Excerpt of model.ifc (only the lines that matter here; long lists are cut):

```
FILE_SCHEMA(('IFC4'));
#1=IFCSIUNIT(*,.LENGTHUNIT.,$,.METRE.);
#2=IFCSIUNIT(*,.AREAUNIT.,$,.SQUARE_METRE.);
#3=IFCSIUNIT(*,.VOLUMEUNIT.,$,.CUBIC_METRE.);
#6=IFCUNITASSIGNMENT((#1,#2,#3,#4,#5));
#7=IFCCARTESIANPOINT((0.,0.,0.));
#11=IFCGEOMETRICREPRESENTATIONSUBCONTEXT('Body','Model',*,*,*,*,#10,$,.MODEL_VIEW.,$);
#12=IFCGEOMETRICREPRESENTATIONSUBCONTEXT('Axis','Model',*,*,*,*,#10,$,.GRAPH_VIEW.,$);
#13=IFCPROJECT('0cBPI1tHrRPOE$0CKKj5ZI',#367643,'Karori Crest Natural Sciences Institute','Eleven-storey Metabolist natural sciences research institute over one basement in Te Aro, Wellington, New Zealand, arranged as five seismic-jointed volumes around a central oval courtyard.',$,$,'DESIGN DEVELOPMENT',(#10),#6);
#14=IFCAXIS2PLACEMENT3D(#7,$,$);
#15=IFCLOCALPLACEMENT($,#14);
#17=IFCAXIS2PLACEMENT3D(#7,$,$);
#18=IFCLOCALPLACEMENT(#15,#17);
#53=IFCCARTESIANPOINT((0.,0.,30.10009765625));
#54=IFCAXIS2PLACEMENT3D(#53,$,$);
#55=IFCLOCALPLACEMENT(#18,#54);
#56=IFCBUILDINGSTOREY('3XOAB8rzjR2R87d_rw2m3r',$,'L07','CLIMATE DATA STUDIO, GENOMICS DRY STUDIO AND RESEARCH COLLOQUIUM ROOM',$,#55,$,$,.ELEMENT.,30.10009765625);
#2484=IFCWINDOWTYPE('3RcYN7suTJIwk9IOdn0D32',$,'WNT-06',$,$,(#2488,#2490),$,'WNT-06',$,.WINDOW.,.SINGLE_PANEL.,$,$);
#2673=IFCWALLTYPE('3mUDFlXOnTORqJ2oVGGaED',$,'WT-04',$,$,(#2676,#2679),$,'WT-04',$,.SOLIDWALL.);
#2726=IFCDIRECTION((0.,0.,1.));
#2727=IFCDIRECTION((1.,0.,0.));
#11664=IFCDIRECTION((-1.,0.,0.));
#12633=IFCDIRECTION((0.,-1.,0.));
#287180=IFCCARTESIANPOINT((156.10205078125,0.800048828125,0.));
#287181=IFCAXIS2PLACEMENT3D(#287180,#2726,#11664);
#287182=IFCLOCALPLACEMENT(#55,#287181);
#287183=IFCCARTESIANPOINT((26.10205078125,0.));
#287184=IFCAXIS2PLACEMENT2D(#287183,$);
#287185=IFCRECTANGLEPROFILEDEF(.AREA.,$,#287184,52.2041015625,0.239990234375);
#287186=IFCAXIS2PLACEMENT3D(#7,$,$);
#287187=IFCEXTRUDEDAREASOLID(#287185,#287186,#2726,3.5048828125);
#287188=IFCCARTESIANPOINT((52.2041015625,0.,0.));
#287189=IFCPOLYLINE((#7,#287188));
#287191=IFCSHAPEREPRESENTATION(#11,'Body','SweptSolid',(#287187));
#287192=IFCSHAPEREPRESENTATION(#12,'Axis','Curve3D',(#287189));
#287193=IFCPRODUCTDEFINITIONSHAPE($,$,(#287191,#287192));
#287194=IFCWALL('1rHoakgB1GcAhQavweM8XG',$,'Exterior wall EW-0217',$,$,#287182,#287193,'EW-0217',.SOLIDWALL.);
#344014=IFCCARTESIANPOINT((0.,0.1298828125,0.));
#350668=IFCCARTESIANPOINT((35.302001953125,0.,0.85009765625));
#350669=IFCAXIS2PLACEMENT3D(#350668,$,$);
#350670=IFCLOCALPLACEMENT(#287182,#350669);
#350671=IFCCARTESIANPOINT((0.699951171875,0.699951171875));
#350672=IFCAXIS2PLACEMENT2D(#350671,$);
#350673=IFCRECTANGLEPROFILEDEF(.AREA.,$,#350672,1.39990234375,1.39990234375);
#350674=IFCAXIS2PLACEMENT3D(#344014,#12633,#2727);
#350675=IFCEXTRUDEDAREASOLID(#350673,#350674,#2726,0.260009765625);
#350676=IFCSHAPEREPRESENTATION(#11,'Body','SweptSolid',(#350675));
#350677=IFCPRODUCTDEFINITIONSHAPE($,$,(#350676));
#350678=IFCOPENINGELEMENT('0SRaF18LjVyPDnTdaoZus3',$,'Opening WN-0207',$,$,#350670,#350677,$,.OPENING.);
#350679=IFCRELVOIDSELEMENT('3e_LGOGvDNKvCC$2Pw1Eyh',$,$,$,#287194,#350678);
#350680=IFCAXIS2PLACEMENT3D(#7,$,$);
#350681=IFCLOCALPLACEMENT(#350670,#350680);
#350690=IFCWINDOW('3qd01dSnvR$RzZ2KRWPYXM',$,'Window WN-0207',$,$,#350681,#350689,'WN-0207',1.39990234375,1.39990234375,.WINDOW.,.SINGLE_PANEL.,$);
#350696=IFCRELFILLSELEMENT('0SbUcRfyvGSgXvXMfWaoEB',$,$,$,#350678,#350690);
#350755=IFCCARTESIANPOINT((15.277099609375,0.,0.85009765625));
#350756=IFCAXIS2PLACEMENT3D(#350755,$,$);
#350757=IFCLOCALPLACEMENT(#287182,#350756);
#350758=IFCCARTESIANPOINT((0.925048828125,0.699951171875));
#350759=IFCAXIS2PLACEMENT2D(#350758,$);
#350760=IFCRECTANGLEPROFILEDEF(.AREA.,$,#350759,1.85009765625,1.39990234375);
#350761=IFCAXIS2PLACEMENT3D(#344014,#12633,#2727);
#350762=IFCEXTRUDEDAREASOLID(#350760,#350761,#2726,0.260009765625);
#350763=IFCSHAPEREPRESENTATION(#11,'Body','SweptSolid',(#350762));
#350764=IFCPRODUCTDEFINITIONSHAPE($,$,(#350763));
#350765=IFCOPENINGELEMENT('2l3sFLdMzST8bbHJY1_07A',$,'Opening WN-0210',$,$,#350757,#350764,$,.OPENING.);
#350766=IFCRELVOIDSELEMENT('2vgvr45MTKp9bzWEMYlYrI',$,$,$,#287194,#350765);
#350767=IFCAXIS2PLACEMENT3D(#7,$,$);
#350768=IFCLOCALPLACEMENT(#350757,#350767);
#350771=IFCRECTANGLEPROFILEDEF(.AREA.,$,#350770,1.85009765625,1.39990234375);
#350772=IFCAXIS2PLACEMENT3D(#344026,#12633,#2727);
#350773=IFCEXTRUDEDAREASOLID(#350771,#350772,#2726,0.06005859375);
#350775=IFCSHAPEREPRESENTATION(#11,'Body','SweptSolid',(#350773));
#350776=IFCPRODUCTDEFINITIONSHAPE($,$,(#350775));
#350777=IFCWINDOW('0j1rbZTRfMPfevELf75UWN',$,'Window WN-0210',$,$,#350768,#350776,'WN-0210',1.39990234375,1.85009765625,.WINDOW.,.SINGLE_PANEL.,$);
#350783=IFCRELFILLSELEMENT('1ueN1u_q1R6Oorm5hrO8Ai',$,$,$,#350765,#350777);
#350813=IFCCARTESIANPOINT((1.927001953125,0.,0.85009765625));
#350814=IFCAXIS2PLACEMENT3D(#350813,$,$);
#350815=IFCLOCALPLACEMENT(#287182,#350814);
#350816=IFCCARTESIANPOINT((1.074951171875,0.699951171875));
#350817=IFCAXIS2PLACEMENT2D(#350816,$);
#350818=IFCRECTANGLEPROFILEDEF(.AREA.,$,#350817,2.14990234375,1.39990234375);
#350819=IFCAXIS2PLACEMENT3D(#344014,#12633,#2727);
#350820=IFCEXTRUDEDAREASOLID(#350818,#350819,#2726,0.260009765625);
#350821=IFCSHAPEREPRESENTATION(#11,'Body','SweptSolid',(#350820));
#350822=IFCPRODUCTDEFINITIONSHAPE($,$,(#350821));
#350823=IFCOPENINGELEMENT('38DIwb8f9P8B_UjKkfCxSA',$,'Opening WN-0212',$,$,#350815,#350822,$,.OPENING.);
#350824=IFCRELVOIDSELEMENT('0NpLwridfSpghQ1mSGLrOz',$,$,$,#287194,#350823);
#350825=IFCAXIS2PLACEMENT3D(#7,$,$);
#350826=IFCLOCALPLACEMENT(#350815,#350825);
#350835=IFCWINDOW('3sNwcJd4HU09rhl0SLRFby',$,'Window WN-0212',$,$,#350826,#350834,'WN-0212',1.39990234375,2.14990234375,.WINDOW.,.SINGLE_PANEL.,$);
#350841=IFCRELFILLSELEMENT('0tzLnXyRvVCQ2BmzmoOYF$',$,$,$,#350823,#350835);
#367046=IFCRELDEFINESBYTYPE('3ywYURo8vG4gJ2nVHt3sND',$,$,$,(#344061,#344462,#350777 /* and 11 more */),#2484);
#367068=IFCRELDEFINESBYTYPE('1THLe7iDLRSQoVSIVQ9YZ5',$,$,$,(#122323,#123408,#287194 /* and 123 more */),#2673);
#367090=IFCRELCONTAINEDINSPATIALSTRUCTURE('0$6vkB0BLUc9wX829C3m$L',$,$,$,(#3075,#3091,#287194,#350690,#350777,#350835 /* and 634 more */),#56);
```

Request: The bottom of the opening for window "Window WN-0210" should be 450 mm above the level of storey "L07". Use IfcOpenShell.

```python
import numpy as np
import ifcopenshell
import ifcopenshell.api.geometry
import ifcopenshell.geom
import ifcopenshell.util.element
import ifcopenshell.util.placement
import ifcopenshell.util.shape
import ifcopenshell.util.unit

model = ifcopenshell.open("model.ifc")
unit_scale = ifcopenshell.util.unit.calculate_unit_scale(model)

window = model.by_guid("0j1rbZTRfMPfevELf75UWN")
opening = window.FillsVoids[0].RelatingOpeningElement
storey = ifcopenshell.util.element.get_container(window, ifc_class="IfcBuildingStorey")
level = ifcopenshell.util.placement.get_local_placement(storey.ObjectPlacement)[2, 3]

# The opening's origin need not be at the sill, so measure its lowest point.
shape = ifcopenshell.geom.create_shape(ifcopenshell.geom.settings(), opening)
bottom = ifcopenshell.util.shape.get_shape_bottom_elevation(shape, shape.geometry) / unit_scale
dz = level + 0.45 / unit_scale - bottom

shift = np.array([0.0, 0.0, dz])
# The window is placed relative to its opening, so it follows when the opening moves.
matrix = ifcopenshell.util.placement.get_local_placement(opening.ObjectPlacement)
matrix[:3, 3] += shift
ifcopenshell.api.geometry.edit_object_placement(
    model, product=opening, matrix=matrix, is_si=False, should_transform_children=True
)

print(f"moved by {dz * unit_scale:+.3f} m")

model.write("model_updated.ifc")
```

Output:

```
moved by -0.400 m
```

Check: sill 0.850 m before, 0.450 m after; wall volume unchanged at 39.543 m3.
